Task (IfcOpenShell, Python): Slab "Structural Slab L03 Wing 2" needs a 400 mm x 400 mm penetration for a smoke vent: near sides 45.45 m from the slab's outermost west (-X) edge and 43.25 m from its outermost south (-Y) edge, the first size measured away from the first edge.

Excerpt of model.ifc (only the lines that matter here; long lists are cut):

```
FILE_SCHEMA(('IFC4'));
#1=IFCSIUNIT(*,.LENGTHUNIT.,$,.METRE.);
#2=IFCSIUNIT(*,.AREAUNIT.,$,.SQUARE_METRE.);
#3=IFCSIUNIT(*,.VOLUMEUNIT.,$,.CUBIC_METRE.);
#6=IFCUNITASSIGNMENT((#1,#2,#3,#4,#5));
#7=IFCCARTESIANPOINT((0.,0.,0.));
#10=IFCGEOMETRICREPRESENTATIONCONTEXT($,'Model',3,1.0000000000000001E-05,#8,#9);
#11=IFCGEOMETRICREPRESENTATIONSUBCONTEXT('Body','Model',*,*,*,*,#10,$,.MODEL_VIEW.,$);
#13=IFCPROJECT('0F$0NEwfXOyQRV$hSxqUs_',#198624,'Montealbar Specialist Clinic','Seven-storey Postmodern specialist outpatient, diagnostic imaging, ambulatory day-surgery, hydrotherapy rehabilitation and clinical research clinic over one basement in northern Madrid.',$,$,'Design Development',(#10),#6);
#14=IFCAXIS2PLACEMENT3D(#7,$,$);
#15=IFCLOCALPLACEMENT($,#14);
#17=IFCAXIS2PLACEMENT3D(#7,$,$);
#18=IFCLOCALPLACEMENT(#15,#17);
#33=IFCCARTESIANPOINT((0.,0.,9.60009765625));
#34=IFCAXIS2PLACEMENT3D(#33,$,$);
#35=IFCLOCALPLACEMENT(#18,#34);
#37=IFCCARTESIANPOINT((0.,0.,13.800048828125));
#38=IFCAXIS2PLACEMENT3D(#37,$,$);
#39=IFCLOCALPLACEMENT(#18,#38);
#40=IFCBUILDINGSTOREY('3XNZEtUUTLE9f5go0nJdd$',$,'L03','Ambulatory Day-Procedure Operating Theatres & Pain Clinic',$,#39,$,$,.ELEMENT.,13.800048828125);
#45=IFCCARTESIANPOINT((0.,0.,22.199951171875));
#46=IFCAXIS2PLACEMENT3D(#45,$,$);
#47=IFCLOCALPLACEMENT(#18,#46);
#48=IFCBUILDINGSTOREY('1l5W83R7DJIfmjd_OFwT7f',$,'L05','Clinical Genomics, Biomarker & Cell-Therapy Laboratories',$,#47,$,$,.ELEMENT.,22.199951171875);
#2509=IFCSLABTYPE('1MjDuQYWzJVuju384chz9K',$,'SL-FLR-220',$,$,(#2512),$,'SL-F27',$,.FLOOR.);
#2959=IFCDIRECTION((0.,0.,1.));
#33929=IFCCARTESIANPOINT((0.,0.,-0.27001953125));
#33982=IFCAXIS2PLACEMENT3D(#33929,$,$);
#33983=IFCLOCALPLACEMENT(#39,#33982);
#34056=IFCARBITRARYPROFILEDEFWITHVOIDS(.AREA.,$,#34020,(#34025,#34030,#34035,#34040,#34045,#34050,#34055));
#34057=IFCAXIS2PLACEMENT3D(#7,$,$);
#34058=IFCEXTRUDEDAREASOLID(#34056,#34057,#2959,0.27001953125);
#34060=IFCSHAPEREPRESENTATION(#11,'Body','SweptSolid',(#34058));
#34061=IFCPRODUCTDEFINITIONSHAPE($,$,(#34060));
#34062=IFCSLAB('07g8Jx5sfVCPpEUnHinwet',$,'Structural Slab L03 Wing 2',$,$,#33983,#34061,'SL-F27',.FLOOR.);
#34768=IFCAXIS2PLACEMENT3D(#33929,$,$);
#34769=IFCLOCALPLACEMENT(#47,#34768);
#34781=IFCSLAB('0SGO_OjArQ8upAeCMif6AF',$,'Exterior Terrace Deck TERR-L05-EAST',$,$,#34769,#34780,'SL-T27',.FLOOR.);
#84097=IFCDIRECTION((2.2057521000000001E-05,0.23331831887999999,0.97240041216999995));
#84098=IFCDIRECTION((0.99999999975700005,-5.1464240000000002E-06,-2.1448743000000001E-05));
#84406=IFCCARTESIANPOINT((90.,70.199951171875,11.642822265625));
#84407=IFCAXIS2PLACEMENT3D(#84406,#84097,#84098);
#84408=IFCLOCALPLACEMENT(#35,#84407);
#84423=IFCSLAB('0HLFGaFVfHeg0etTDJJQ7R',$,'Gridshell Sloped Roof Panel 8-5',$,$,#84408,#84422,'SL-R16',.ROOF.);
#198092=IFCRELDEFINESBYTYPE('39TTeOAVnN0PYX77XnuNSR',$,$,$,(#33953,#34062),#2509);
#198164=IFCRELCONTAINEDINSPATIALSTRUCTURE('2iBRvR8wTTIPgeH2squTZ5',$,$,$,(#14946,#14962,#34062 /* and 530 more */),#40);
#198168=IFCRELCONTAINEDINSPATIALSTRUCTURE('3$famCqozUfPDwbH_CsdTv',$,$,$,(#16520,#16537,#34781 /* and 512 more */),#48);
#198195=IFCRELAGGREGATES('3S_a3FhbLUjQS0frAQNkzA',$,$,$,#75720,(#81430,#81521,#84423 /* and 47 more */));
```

```python
import numpy as np
import ifcopenshell
import ifcopenshell.api.feature
import ifcopenshell.api.geometry
import ifcopenshell.api.root
import ifcopenshell.geom
import ifcopenshell.util.placement
import ifcopenshell.util.representation
import ifcopenshell.util.shape
import ifcopenshell.util.unit

model = ifcopenshell.open("model.ifc")
unit_scale = ifcopenshell.util.unit.calculate_unit_scale(model)
settings = ifcopenshell.geom.settings()


def volume(element):
    """Net volume in cubic metres, openings subtracted."""
    shape = ifcopenshell.geom.create_shape(settings, element)
    return ifcopenshell.util.shape.get_volume(shape.geometry)


slab = model.by_id(34062)
before = volume(slab)

# Extent in the slab's own axes, in metres. The edges named are its -X and -Y sides.
slab_shape = ifcopenshell.geom.create_shape(settings, slab)
vertices = ifcopenshell.util.shape.get_vertices(slab_shape.geometry)
x_min, y_min, bottom = vertices.min(axis=0)
top = vertices[:, 2].max()

opening = ifcopenshell.api.root.create_entity(model, ifc_class="IfcOpeningElement", name="Smoke vent opening", predefined_type="OPENING")
context = ifcopenshell.util.representation.get_context(model, "Model", "Body", "MODEL_VIEW")
width, depth = 0.4, 0.4
outline = [(0.0, 0.0), (width, 0.0), (width, depth), (0.0, depth), (0.0, 0.0)]
# Overshoot both faces by 50 mm so the cut is clean.
shape = ifcopenshell.api.geometry.add_slab_representation(
    model, context=context, depth=top - bottom + 0.1, polyline=outline
)
ifcopenshell.api.geometry.assign_representation(model, product=opening, representation=shape)

matrix = ifcopenshell.util.placement.get_local_placement(slab.ObjectPlacement)
matrix[:, 3] = matrix @ np.append(np.array([x_min + 45.45, y_min + 43.25, bottom - 0.05]) / unit_scale, 1.0)
ifcopenshell.api.geometry.edit_object_placement(model, product=opening, matrix=matrix, is_si=False)
ifcopenshell.api.feature.add_feature(model, feature=opening, element=slab)

after = volume(slab)

print(f"slab volume {before:.3f} -> {after:.3f} m3")

model.write("model_rev.ifc")
```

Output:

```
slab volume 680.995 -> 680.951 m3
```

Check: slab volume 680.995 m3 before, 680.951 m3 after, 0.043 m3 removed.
